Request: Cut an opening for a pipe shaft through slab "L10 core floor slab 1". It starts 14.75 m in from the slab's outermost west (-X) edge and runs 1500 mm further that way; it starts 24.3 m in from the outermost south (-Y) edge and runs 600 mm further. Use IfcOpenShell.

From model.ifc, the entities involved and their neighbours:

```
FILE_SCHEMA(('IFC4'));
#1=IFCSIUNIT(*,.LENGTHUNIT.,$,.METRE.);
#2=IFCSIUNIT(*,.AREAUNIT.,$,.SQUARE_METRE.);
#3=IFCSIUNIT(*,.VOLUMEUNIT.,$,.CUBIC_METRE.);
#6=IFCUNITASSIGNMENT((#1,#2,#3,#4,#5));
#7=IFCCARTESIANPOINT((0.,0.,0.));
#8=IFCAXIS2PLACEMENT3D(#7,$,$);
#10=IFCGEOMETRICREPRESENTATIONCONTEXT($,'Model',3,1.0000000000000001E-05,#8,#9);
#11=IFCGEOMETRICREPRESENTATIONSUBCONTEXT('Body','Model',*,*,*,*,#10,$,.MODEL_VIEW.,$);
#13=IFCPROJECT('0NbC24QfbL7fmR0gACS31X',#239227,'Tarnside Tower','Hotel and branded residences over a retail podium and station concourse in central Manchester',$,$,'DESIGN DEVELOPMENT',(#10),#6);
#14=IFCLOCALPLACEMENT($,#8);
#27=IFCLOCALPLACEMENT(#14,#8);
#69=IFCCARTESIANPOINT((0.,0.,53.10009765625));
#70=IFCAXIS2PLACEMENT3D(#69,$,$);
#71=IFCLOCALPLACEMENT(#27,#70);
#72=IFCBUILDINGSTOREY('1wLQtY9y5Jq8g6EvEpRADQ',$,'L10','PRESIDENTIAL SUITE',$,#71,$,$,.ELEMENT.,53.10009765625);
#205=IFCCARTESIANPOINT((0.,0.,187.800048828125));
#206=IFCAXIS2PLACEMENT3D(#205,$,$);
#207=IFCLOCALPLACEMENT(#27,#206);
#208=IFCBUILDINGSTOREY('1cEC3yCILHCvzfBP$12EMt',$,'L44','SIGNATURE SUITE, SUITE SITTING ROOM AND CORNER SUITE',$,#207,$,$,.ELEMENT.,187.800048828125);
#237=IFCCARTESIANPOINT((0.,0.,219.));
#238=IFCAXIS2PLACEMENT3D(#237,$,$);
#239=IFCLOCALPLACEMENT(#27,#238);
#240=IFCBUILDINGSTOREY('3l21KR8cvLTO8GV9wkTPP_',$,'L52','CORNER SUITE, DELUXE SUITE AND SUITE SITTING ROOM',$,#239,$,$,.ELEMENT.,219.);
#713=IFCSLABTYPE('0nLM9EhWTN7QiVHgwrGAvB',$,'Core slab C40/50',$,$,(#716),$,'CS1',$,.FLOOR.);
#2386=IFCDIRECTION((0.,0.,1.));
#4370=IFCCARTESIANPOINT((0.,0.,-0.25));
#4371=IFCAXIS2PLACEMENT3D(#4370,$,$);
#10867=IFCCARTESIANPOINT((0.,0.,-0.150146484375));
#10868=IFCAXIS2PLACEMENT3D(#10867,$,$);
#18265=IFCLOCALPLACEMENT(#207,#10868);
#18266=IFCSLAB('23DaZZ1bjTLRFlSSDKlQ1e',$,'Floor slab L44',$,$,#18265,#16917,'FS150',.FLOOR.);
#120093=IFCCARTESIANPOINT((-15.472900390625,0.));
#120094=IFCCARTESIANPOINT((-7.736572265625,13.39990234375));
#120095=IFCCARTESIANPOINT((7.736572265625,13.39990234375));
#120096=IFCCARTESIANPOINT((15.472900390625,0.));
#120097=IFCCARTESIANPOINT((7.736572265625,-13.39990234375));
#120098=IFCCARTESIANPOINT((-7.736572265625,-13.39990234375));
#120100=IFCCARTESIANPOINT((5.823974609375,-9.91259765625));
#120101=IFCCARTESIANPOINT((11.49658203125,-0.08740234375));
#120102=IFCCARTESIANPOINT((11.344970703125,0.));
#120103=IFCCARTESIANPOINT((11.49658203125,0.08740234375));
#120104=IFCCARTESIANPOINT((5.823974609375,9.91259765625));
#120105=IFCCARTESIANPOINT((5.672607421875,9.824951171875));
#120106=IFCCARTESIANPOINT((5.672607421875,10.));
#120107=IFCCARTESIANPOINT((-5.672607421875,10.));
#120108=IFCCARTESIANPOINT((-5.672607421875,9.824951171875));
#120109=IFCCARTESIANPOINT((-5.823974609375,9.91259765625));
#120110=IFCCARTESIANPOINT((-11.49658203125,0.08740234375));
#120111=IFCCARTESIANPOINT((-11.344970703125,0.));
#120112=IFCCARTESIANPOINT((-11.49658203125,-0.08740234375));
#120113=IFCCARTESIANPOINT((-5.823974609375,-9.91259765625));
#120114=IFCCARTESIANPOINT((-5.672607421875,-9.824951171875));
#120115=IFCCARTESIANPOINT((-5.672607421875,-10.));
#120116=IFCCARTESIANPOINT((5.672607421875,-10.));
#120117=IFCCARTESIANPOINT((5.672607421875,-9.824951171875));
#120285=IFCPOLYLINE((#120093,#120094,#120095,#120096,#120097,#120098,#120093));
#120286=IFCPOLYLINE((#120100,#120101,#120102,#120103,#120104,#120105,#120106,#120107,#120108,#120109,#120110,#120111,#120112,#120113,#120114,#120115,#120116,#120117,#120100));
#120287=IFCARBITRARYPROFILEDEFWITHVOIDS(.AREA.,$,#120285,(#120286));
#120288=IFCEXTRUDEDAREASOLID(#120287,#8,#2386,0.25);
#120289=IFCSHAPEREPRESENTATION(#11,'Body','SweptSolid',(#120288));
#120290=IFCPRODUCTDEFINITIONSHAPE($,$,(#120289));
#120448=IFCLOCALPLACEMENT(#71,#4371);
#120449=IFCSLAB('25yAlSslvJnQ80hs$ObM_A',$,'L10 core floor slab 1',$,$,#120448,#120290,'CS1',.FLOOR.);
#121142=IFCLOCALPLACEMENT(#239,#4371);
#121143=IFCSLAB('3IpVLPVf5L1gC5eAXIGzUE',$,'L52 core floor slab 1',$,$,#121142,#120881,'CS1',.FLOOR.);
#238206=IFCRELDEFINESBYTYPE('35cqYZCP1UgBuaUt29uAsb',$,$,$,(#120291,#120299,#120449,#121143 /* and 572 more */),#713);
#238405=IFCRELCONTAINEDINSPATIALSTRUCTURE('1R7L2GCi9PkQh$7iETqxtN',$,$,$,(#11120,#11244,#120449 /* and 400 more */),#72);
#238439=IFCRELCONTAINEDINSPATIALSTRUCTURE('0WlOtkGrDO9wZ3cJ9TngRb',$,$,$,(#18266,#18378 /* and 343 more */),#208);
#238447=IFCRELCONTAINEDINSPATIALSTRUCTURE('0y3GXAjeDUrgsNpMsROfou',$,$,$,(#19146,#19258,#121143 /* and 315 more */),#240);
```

```python
import numpy as np
import ifcopenshell
import ifcopenshell.api.feature
import ifcopenshell.api.geometry
import ifcopenshell.api.root
import ifcopenshell.geom
import ifcopenshell.util.placement
import ifcopenshell.util.representation
import ifcopenshell.util.shape
import ifcopenshell.util.unit

model = ifcopenshell.open("model.ifc")
unit_scale = ifcopenshell.util.unit.calculate_unit_scale(model)
settings = ifcopenshell.geom.settings()


def volume(element):
    """Net volume in cubic metres, openings subtracted."""
    shape = ifcopenshell.geom.create_shape(settings, element)
    return ifcopenshell.util.shape.get_volume(shape.geometry)


slab = model.by_id(120449)
before = volume(slab)

# Extent in the slab's own axes, in metres. The edges named are its -X and -Y sides.
slab_shape = ifcopenshell.geom.create_shape(settings, slab)
vertices = ifcopenshell.util.shape.get_vertices(slab_shape.geometry)
x_min, y_min, bottom = vertices.min(axis=0)
top = vertices[:, 2].max()

opening = ifcopenshell.api.root.create_entity(model, ifc_class="IfcOpeningElement", name="Pipe shaft opening", predefined_type="OPENING")
context = ifcopenshell.util.representation.get_context(model, "Model", "Body", "MODEL_VIEW")
width, depth = 1.5, 0.6
outline = [(0.0, 0.0), (width, 0.0), (width, depth), (0.0, depth), (0.0, 0.0)]
# Overshoot both faces by 50 mm so the cut is clean.
shape = ifcopenshell.api.geometry.add_slab_representation(
    model, context=context, depth=top - bottom + 0.1, polyline=outline
)
ifcopenshell.api.geometry.assign_representation(model, product=opening, representation=shape)

matrix = ifcopenshell.util.placement.get_local_placement(slab.ObjectPlacement)
matrix[:, 3] = matrix @ np.append(np.array([x_min + 14.75, y_min + 24.3, bottom - 0.05]) / unit_scale, 1.0)
ifcopenshell.api.geometry.edit_object_placement(model, product=opening, matrix=matrix, is_si=False)
ifcopenshell.api.feature.add_feature(model, feature=opening, element=slab)

after = volume(slab)

print(f"slab volume {before:.3f} -> {after:.3f} m3")

model.write("model_edited.ifc")
```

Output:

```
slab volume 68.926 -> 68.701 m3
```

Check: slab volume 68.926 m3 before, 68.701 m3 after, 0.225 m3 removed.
